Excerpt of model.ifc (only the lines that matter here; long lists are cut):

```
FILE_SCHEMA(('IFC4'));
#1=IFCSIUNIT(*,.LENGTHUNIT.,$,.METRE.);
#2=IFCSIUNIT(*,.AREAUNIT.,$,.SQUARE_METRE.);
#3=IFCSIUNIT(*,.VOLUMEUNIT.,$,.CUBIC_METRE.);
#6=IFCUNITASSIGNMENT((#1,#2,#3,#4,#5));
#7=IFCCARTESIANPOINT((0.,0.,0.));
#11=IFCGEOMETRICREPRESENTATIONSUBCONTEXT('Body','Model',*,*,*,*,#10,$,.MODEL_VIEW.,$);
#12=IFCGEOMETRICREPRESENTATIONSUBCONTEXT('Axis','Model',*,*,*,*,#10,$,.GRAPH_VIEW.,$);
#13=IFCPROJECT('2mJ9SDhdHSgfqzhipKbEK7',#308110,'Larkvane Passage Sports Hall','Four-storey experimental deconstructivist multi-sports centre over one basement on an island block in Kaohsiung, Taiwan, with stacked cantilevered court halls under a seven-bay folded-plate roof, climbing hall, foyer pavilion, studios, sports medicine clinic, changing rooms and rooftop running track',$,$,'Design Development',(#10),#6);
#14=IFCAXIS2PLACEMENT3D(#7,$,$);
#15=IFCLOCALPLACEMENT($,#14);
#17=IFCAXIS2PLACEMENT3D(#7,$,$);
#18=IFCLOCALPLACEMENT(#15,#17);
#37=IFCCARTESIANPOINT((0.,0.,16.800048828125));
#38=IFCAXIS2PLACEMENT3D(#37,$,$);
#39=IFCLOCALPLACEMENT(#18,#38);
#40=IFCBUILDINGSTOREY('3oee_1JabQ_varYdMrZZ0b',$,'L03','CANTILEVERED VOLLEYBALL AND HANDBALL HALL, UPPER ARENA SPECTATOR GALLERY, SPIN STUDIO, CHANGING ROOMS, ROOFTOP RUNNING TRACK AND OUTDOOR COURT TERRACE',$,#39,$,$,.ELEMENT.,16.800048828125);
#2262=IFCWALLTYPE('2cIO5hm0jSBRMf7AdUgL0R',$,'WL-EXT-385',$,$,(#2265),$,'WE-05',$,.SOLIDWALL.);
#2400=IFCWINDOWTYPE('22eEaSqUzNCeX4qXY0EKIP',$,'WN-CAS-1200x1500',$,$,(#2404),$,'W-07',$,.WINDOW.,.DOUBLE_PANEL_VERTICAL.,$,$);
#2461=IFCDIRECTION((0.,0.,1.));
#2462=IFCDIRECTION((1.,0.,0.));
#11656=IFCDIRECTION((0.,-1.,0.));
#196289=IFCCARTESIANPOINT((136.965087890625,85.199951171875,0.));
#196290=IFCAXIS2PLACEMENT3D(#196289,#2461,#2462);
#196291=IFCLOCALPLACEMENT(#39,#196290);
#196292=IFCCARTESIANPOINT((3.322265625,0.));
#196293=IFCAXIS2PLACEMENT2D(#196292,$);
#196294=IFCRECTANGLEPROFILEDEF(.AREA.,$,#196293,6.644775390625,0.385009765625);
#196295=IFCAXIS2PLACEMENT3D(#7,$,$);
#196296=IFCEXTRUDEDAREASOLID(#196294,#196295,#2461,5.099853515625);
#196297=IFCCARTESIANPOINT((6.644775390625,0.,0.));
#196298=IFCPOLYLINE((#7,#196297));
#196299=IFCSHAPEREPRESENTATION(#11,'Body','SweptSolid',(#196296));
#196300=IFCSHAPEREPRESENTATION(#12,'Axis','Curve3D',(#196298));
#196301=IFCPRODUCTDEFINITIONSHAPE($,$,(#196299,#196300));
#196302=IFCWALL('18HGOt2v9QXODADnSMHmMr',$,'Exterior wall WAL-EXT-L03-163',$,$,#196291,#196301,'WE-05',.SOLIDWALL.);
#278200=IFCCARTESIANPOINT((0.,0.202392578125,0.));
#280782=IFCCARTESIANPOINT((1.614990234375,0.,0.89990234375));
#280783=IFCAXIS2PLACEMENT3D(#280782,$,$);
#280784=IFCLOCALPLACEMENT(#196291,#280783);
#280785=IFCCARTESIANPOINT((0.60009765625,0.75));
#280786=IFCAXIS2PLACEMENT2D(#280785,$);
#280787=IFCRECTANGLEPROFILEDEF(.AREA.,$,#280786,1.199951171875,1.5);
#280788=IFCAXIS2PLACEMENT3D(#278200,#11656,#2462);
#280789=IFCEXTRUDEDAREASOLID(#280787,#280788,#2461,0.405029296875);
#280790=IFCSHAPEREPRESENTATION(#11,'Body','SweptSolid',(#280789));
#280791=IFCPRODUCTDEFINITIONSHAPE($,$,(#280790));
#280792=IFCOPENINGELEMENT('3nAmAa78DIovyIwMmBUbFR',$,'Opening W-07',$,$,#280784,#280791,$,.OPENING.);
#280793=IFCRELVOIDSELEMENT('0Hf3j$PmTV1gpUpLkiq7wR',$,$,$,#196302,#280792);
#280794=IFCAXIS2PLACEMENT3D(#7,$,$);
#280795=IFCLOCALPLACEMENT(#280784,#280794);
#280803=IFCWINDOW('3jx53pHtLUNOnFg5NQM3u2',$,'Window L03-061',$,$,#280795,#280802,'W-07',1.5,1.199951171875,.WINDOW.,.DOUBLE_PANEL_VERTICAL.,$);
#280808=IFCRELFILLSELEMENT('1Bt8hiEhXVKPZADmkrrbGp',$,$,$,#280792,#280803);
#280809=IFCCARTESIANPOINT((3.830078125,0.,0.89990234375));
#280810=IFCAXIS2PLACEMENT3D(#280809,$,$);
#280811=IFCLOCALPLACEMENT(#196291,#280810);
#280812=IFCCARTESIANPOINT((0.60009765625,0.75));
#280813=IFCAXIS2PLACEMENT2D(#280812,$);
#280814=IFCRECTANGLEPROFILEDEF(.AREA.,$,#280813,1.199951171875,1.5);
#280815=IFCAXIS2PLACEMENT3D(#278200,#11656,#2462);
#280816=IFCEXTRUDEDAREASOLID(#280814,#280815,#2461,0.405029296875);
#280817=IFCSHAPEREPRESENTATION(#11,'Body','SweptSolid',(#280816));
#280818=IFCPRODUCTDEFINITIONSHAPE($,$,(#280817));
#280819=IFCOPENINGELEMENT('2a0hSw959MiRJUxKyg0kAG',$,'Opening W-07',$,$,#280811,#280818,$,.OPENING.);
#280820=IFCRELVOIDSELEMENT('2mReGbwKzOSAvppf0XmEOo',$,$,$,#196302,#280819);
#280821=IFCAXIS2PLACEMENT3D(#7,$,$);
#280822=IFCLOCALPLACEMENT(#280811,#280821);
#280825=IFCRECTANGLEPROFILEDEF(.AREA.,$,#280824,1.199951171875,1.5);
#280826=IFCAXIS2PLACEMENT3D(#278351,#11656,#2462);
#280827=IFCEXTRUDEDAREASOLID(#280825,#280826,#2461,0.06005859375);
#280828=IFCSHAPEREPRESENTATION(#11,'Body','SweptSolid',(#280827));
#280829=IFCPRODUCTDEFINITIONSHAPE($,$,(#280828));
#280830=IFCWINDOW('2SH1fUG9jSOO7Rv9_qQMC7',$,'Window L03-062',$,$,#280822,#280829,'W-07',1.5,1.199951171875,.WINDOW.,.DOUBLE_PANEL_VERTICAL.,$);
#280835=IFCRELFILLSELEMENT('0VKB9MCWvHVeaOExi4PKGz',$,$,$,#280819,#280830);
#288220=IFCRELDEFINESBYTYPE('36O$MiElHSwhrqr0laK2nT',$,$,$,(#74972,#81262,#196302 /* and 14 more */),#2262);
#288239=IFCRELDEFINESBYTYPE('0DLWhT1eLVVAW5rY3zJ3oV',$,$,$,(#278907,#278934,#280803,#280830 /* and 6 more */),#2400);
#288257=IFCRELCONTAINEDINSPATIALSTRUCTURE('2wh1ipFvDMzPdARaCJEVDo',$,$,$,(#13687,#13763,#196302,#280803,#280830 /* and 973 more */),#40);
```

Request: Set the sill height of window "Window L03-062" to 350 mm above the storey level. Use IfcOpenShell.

```python
import numpy as np
import ifcopenshell
import ifcopenshell.api.geometry
import ifcopenshell.geom
import ifcopenshell.util.element
import ifcopenshell.util.placement
import ifcopenshell.util.shape
import ifcopenshell.util.unit

model = ifcopenshell.open("model.ifc")
unit_scale = ifcopenshell.util.unit.calculate_unit_scale(model)

window = model.by_id(280830)
opening = window.FillsVoids[0].RelatingOpeningElement
storey = ifcopenshell.util.element.get_container(window, ifc_class="IfcBuildingStorey")
level = ifcopenshell.util.placement.get_local_placement(storey.ObjectPlacement)[2, 3]

# The opening's origin need not be at the sill, so measure its lowest point.
shape = ifcopenshell.geom.create_shape(ifcopenshell.geom.settings(), opening)
bottom = ifcopenshell.util.shape.get_shape_bottom_elevation(shape, shape.geometry) / unit_scale
dz = level + 0.35 - bottom

shift = np.array([0.0, 0.0, dz])
# The window is placed relative to its opening, so it follows when the opening moves.
matrix = ifcopenshell.util.placement.get_local_placement(opening.ObjectPlacement)
matrix[:3, 3] += shift
ifcopenshell.api.geometry.edit_object_placement(
    model, product=opening, matrix=matrix, is_si=False, should_transform_children=True
)

print(f"moved by {dz * unit_scale:+.3f} m")

model.write("model_edited.ifc")
```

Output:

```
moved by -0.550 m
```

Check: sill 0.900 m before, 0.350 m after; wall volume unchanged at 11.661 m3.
